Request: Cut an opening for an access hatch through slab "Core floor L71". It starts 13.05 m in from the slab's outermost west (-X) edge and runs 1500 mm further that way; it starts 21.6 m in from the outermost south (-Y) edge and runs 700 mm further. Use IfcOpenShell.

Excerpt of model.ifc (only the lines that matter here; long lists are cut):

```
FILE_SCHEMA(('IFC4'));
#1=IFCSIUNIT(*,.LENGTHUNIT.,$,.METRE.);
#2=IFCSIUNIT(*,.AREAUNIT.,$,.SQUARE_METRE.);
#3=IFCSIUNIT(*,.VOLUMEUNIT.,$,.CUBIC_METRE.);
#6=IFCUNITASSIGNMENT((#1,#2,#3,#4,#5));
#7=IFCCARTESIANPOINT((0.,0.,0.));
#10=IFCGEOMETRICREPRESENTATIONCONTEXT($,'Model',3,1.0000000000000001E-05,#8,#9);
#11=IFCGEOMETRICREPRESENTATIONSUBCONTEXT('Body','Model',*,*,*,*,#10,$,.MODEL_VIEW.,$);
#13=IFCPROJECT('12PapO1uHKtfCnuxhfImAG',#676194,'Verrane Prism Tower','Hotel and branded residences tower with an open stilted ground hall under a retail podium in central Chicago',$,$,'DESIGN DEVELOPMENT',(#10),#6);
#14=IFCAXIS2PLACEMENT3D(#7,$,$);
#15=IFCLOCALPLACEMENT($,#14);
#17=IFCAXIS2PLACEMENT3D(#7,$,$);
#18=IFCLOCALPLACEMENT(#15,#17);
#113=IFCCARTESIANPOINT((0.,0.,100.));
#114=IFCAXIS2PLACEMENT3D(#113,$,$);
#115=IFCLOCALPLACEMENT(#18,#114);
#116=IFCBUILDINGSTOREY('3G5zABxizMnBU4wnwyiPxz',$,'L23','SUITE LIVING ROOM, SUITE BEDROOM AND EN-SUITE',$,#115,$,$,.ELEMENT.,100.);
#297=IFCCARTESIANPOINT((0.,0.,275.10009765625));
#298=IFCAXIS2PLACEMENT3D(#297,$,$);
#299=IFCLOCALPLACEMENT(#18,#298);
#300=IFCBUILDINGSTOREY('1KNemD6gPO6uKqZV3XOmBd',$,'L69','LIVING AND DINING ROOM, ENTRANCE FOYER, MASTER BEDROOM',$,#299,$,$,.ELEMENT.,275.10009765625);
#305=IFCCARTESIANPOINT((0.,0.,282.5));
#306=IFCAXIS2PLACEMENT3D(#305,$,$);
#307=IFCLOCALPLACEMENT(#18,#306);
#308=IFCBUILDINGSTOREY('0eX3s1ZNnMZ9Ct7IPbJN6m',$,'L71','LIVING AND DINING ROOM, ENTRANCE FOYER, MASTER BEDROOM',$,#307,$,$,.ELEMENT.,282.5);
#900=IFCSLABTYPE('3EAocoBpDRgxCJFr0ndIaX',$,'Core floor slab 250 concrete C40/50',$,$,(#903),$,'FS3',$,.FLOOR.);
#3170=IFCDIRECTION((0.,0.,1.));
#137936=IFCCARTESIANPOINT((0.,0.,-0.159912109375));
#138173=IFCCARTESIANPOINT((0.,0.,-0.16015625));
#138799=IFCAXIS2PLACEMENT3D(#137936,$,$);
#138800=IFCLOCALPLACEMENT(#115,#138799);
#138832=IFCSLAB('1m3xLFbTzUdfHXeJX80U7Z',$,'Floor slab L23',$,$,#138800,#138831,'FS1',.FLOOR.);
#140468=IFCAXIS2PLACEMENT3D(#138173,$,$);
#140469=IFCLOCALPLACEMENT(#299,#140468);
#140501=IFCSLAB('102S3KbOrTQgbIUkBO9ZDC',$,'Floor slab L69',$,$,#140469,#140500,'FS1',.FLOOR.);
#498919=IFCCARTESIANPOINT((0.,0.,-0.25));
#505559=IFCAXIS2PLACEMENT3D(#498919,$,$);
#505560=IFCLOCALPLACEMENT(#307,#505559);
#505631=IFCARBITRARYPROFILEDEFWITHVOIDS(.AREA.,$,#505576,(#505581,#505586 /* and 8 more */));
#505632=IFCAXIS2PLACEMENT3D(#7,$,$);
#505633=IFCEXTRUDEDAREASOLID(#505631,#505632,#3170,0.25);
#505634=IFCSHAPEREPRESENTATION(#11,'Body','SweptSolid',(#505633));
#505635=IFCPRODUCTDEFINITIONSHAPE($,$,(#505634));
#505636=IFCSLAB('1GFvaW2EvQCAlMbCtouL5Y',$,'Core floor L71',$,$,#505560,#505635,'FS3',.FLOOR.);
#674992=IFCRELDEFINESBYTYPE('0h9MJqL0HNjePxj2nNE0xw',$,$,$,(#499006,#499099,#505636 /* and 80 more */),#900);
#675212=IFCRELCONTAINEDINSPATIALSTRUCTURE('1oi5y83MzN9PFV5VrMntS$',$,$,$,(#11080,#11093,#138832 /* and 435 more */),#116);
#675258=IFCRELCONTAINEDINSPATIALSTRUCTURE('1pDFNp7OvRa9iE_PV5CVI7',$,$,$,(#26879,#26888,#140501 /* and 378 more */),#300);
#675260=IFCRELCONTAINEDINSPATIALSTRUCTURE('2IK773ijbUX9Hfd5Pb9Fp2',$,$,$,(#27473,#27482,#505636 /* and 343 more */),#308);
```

```python
import numpy as np
import ifcopenshell
import ifcopenshell.api.feature
import ifcopenshell.api.geometry
import ifcopenshell.api.root
import ifcopenshell.geom
import ifcopenshell.util.placement
import ifcopenshell.util.representation
import ifcopenshell.util.shape
import ifcopenshell.util.unit

model = ifcopenshell.open("model.ifc")
unit_scale = ifcopenshell.util.unit.calculate_unit_scale(model)
settings = ifcopenshell.geom.settings()


def volume(element):
    """Net volume in cubic metres, openings subtracted."""
    shape = ifcopenshell.geom.create_shape(settings, element)
    return ifcopenshell.util.shape.get_volume(shape.geometry)


slab = model.by_id(505636)
before = volume(slab)

# Extent in the slab's own axes, in metres. The edges named are its -X and -Y sides.
slab_shape = ifcopenshell.geom.create_shape(settings, slab)
vertices = ifcopenshell.util.shape.get_vertices(slab_shape.geometry)
x_min, y_min, bottom = vertices.min(axis=0)
top = vertices[:, 2].max()

opening = ifcopenshell.api.root.create_entity(model, ifc_class="IfcOpeningElement", name="Access hatch opening", predefined_type="OPENING")
context = ifcopenshell.util.representation.get_context(model, "Model", "Body", "MODEL_VIEW")
width, depth = 1.5, 0.7
outline = [(0.0, 0.0), (width, 0.0), (width, depth), (0.0, depth), (0.0, 0.0)]
# Overshoot both faces by 50 mm so the cut is clean.
shape = ifcopenshell.api.geometry.add_slab_representation(
    model, context=context, depth=top - bottom + 0.1, polyline=outline
)
ifcopenshell.api.geometry.assign_representation(model, product=opening, representation=shape)

matrix = ifcopenshell.util.placement.get_local_placement(slab.ObjectPlacement)
matrix[:, 3] = matrix @ np.append(np.array([x_min + 13.05, y_min + 21.6, bottom - 0.05]) / unit_scale, 1.0)
ifcopenshell.api.geometry.edit_object_placement(model, product=opening, matrix=matrix, is_si=False)
ifcopenshell.api.feature.add_feature(model, feature=opening, element=slab)

after = volume(slab)

print(f"slab volume {before:.3f} -> {after:.3f} m3")

model.write("model_v2.ifc")
```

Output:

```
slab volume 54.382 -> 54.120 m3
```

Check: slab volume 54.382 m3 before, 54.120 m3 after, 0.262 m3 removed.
